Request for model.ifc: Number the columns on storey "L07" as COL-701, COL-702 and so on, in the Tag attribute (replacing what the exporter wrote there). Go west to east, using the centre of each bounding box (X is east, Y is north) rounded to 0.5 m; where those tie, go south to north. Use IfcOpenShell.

First a look at what the model holds.

```python
import ifcopenshell
import ifcopenshell.util.element
import ifcopenshell.util.placement

model = ifcopenshell.open("model.ifc")
print(model.schema)
storey = next(s for s in model.by_type("IfcBuildingStorey") if s.Name == "L07")
columns = [e for e in ifcopenshell.util.element.get_decomposition(storey) if e.is_a("IfcColumn")]
for e in sorted(columns, key=lambda e: e.id()):
    origin = ifcopenshell.util.placement.get_local_placement(e.ObjectPlacement)[:3, 3]
    print(e.id(), e.Tag, e.Name, origin.round(2) + 0.0, sep=" | ")
```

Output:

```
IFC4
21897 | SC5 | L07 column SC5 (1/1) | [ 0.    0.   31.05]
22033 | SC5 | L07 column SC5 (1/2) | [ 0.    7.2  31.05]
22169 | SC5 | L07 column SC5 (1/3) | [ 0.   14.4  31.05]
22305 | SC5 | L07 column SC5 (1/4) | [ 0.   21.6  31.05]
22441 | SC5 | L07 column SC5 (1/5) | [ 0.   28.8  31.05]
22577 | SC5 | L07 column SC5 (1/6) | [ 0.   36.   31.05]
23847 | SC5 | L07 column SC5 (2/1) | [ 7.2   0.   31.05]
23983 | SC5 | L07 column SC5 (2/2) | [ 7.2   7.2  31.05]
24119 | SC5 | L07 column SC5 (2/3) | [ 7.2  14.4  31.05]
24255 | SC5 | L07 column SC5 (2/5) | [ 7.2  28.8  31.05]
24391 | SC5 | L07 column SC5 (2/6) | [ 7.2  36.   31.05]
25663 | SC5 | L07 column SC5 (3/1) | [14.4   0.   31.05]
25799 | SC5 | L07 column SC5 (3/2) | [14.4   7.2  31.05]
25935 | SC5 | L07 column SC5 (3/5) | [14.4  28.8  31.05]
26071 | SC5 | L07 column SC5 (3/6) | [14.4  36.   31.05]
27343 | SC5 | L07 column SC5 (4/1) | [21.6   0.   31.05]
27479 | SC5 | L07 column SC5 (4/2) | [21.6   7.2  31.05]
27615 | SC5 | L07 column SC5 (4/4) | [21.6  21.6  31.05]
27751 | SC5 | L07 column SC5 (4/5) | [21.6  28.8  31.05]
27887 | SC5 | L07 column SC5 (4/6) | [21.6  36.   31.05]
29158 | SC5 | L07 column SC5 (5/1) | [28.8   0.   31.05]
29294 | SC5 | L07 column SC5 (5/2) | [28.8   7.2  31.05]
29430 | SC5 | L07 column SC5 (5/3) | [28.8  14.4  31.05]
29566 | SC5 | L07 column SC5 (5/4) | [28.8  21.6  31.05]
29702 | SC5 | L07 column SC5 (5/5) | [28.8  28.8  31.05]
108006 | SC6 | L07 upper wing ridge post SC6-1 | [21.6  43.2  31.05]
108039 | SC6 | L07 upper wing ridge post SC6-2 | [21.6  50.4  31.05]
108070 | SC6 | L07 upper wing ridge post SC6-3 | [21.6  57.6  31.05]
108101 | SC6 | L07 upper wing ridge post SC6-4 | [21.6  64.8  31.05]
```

```python
import ifcopenshell
import ifcopenshell.geom
import ifcopenshell.util.element
import ifcopenshell.util.shape

model = ifcopenshell.open("model.ifc")
settings = ifcopenshell.geom.settings()
settings.set("use-world-coords", True)


def centre(element):
    shape = ifcopenshell.geom.create_shape(settings, element)
    return ifcopenshell.util.shape.get_bbox_centroid(shape.geometry)


storey = next(s for s in model.by_type("IfcBuildingStorey") if s.Name == "L07")
columns = [e for e in ifcopenshell.util.element.get_decomposition(storey) if e.is_a("IfcColumn")]

# Insertion points can sit at a corner or the storey origin, so sort by the geometry (in metres).
centres = {e: centre(e) for e in columns}
columns.sort(key=lambda e: (round(centres[e][0] / 0.5), centres[e][1]))

for i, e in enumerate(columns, start=1):
    number = f"COL-7{i:02d}"
    e.Tag = number
    print(e.id(), number)

model.write("model_updated.ifc")
```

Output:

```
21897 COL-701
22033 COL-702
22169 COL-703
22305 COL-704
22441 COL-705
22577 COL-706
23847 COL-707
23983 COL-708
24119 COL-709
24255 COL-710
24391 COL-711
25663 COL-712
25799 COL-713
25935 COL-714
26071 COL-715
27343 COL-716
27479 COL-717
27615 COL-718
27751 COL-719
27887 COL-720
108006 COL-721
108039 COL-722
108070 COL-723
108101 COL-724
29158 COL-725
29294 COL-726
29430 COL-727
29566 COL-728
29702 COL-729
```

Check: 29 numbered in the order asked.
